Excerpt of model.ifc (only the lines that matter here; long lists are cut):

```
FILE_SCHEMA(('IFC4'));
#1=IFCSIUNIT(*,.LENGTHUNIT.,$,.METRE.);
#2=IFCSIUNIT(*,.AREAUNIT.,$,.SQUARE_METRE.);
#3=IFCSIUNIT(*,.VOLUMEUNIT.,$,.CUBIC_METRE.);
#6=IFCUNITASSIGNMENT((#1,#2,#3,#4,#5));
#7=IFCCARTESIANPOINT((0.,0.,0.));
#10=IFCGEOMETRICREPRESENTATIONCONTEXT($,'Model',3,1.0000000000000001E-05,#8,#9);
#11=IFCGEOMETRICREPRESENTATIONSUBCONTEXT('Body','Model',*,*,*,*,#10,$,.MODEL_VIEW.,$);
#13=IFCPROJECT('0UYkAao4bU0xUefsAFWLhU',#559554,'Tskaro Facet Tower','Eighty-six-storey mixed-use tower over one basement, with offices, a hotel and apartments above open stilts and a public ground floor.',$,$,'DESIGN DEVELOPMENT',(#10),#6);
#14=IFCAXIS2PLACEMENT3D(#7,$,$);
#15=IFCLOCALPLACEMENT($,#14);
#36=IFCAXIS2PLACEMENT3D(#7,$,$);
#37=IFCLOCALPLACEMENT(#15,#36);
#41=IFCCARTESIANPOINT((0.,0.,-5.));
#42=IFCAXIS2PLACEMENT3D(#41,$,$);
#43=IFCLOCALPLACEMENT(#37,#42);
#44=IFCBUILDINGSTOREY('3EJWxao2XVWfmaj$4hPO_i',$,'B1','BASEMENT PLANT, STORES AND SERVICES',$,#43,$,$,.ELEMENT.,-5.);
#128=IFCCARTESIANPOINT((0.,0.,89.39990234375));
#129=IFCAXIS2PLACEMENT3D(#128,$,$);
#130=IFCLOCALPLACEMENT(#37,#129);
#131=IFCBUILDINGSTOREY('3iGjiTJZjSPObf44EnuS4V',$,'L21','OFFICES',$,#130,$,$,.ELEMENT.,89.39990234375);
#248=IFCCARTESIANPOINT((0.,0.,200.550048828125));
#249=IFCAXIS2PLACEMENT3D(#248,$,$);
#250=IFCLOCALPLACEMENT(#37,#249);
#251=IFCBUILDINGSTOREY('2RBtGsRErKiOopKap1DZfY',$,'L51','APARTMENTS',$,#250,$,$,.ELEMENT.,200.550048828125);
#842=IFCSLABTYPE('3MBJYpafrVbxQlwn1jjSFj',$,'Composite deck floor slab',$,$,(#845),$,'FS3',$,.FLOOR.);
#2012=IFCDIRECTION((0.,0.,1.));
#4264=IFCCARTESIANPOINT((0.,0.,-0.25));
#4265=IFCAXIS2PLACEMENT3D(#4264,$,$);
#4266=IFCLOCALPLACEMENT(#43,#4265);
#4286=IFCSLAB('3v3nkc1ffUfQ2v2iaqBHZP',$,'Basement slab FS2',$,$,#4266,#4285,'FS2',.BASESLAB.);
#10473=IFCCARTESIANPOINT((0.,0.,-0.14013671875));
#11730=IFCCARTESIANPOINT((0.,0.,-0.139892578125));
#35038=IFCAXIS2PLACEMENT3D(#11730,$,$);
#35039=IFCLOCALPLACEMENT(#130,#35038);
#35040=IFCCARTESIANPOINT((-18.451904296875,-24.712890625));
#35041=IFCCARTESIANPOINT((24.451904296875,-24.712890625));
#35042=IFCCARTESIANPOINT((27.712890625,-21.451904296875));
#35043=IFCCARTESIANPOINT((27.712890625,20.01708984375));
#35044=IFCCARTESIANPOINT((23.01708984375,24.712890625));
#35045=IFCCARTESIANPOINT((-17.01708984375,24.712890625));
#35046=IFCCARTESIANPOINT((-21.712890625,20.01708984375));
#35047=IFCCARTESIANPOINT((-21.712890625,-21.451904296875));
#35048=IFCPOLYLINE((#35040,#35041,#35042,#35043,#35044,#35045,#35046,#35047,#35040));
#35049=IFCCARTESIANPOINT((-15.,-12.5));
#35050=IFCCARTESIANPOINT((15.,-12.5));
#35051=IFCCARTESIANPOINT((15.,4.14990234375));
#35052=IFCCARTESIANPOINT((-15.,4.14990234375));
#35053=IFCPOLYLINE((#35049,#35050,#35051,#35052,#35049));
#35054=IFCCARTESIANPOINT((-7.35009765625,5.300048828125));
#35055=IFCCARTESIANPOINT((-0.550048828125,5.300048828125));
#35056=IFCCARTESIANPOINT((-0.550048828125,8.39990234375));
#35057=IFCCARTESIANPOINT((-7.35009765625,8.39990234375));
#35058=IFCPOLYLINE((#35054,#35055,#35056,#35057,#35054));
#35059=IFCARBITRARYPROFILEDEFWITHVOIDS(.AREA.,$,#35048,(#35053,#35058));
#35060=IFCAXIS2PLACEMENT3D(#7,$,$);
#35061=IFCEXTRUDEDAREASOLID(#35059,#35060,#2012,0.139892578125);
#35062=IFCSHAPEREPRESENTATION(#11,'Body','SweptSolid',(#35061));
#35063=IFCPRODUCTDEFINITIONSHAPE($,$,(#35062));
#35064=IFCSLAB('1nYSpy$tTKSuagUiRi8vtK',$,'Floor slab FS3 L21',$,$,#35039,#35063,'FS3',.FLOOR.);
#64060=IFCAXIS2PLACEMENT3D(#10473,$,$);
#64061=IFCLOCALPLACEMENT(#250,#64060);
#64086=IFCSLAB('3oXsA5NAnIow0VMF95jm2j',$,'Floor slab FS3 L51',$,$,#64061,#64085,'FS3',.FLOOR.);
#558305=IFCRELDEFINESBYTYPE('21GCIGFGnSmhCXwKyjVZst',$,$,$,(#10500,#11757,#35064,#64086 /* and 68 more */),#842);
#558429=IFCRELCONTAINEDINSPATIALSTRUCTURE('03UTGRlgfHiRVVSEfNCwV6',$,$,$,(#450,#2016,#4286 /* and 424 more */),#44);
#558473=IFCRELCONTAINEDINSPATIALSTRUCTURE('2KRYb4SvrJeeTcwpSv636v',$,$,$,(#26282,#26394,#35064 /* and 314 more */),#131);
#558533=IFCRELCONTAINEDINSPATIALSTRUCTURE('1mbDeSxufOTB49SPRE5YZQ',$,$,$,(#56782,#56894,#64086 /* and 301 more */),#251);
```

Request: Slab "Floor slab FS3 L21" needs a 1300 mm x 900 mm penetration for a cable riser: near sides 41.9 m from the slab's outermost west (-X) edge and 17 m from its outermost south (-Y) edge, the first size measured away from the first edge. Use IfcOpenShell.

```python
import numpy as np
import ifcopenshell
import ifcopenshell.api.feature
import ifcopenshell.api.geometry
import ifcopenshell.api.root
import ifcopenshell.geom
import ifcopenshell.util.placement
import ifcopenshell.util.representation
import ifcopenshell.util.shape
import ifcopenshell.util.unit

model = ifcopenshell.open("model.ifc")
unit_scale = ifcopenshell.util.unit.calculate_unit_scale(model)
settings = ifcopenshell.geom.settings()


def volume(element):
    """Net volume in cubic metres, openings subtracted."""
    shape = ifcopenshell.geom.create_shape(settings, element)
    return ifcopenshell.util.shape.get_volume(shape.geometry)


slab = model.by_guid("1nYSpy$tTKSuagUiRi8vtK")
before = volume(slab)

# Extent in the slab's own axes, in metres. The edges named are its -X and -Y sides.
slab_shape = ifcopenshell.geom.create_shape(settings, slab)
vertices = ifcopenshell.util.shape.get_vertices(slab_shape.geometry)
x_min, y_min, bottom = vertices.min(axis=0)
top = vertices[:, 2].max()

opening = ifcopenshell.api.root.create_entity(model, ifc_class="IfcOpeningElement", name="Cable riser opening", predefined_type="OPENING")
context = ifcopenshell.util.representation.get_context(model, "Model", "Body", "MODEL_VIEW")
width, depth = 1.3, 0.9
outline = [(0.0, 0.0), (width, 0.0), (width, depth), (0.0, depth), (0.0, 0.0)]
# Overshoot both faces by 50 mm so the cut is clean.
shape = ifcopenshell.api.geometry.add_slab_representation(
    model, context=context, depth=top - bottom + 0.1, polyline=outline
)
ifcopenshell.api.geometry.assign_representation(model, product=opening, representation=shape)

matrix = ifcopenshell.util.placement.get_local_placement(slab.ObjectPlacement)
matrix[:, 3] = matrix @ np.append(np.array([x_min + 41.9, y_min + 17, bottom - 0.05]) / unit_scale, 1.0)
ifcopenshell.api.geometry.edit_object_placement(model, product=opening, matrix=matrix, is_si=False)
ifcopenshell.api.feature.add_feature(model, feature=opening, element=slab)

after = volume(slab)

print(f"slab volume {before:.3f} -> {after:.3f} m3")

model.write("model_updated.ifc")
```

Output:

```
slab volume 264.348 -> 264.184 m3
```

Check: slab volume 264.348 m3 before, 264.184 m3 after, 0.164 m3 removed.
